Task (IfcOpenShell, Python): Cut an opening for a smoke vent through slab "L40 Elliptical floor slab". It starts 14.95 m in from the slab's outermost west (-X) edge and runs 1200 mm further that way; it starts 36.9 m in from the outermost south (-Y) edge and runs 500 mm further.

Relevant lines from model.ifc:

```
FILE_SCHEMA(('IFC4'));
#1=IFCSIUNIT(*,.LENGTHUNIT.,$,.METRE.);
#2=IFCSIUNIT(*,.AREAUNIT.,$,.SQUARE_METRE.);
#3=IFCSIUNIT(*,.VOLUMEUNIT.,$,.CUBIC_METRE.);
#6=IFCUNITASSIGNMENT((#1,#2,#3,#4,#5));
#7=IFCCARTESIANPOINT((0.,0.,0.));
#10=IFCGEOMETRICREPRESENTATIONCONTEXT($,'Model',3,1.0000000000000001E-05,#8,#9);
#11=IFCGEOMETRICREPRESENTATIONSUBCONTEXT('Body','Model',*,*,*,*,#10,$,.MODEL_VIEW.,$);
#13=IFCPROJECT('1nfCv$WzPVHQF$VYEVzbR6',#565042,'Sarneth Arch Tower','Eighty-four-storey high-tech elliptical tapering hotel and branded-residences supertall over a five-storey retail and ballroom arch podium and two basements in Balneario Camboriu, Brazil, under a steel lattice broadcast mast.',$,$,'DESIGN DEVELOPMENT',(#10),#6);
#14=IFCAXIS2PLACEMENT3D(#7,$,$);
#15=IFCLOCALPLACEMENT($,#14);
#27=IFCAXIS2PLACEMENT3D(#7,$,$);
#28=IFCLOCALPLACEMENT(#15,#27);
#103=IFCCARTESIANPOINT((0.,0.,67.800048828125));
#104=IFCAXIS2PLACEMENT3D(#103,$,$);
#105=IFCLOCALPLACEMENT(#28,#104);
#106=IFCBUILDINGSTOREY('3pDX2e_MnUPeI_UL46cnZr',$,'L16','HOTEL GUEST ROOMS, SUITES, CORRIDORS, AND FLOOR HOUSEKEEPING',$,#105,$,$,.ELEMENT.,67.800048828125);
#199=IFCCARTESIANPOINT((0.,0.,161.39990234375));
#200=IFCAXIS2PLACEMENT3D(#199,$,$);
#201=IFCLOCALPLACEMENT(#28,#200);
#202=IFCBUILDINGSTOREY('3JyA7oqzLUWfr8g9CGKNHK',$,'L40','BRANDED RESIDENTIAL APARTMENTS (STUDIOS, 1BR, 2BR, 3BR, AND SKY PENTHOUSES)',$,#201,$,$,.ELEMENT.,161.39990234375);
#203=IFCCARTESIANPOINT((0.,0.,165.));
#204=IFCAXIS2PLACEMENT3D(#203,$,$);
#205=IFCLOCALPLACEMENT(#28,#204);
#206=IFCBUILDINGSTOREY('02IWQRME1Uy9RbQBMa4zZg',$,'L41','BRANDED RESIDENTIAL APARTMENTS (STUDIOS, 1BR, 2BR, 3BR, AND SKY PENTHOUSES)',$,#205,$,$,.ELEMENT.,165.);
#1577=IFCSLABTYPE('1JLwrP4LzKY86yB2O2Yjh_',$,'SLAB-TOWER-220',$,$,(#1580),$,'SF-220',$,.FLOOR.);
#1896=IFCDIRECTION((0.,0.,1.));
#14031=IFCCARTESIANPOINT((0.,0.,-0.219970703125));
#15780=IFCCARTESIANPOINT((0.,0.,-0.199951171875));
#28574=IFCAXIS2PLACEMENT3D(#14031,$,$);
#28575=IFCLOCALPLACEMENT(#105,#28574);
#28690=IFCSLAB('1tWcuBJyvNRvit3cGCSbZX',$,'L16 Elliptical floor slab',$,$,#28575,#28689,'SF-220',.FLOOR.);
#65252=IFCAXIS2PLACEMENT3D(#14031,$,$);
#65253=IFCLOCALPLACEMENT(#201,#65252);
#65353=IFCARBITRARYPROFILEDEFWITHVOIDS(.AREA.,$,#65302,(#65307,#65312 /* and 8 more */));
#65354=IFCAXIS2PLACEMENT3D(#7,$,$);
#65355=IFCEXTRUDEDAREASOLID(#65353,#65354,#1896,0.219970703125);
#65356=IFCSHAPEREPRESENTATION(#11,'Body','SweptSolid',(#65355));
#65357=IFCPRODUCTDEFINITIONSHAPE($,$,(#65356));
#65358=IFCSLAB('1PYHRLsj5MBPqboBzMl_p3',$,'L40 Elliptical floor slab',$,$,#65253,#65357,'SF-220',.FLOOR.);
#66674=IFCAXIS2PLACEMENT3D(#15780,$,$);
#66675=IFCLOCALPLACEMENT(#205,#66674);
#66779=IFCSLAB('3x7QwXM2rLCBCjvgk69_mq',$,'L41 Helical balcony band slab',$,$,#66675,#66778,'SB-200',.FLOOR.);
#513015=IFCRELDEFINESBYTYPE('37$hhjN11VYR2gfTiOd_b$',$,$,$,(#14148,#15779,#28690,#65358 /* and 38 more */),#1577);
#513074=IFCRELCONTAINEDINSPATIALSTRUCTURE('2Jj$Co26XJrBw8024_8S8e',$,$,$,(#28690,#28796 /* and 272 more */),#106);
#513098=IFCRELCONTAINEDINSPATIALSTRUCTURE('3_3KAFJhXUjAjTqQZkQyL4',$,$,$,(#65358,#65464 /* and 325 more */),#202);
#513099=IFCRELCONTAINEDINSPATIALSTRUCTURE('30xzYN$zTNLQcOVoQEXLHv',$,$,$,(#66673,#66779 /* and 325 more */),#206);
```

```python
import numpy as np
import ifcopenshell
import ifcopenshell.api.feature
import ifcopenshell.api.geometry
import ifcopenshell.api.root
import ifcopenshell.geom
import ifcopenshell.util.placement
import ifcopenshell.util.representation
import ifcopenshell.util.shape
import ifcopenshell.util.unit

model = ifcopenshell.open("model.ifc")
unit_scale = ifcopenshell.util.unit.calculate_unit_scale(model)
settings = ifcopenshell.geom.settings()


def volume(element):
    """Net volume in cubic metres, openings subtracted."""
    shape = ifcopenshell.geom.create_shape(settings, element)
    return ifcopenshell.util.shape.get_volume(shape.geometry)


slab = model.by_id(65358)
before = volume(slab)

# Extent in the slab's own axes, in metres. The edges named are its -X and -Y sides.
slab_shape = ifcopenshell.geom.create_shape(settings, slab)
vertices = ifcopenshell.util.shape.get_vertices(slab_shape.geometry)
x_min, y_min, bottom = vertices.min(axis=0)
top = vertices[:, 2].max()

opening = ifcopenshell.api.root.create_entity(model, ifc_class="IfcOpeningElement", name="Smoke vent opening", predefined_type="OPENING")
context = ifcopenshell.util.representation.get_context(model, "Model", "Body", "MODEL_VIEW")
width, depth = 1.2, 0.5
outline = [(0.0, 0.0), (width, 0.0), (width, depth), (0.0, depth), (0.0, 0.0)]
# Overshoot both faces by 50 mm so the cut is clean.
shape = ifcopenshell.api.geometry.add_slab_representation(
    model, context=context, depth=top - bottom + 0.1, polyline=outline
)
ifcopenshell.api.geometry.assign_representation(model, product=opening, representation=shape)

matrix = ifcopenshell.util.placement.get_local_placement(slab.ObjectPlacement)
matrix[:, 3] = matrix @ np.append(np.array([x_min + 14.95, y_min + 36.9, bottom - 0.05]) / unit_scale, 1.0)
ifcopenshell.api.geometry.edit_object_placement(model, product=opening, matrix=matrix, is_si=False)
ifcopenshell.api.feature.add_feature(model, feature=opening, element=slab)

after = volume(slab)

print(f"slab volume {before:.3f} -> {after:.3f} m3")

model.write("model_updated.ifc")
```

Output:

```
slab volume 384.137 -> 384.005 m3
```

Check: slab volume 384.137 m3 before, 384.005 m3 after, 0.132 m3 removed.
